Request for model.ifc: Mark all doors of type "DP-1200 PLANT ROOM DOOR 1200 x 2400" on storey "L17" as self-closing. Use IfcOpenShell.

First a look at what the model holds.

```python
import ifcopenshell
import ifcopenshell.util.element

model = ifcopenshell.open("model.ifc")
print(model.schema)
storey = next(s for s in model.by_type("IfcBuildingStorey") if s.Name == "L17")
doors = [e for e in ifcopenshell.util.element.get_decomposition(storey) if e.is_a("IfcDoor")]
seen = {}
for e in doors:
    element_type = ifcopenshell.util.element.get_type(e)
    key = (element_type.Name if element_type != e and element_type else None, ifcopenshell.util.element.get_pset(e, "Pset_DoorCommon", "SelfClosing"))
    seen[key] = seen.get(key, 0) + 1
for (name, value), count in sorted(seen.items(), key=str):
    print(count, "x", name, "|", value)
```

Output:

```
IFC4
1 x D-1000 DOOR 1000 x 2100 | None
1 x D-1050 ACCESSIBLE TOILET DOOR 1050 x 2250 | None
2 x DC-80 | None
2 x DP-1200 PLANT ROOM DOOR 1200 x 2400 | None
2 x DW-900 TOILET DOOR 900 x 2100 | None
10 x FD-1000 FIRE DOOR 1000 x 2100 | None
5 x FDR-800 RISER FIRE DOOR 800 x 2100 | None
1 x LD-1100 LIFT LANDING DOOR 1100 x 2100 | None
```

```python
import ifcopenshell
import ifcopenshell.api.pset
import ifcopenshell.util.element

model = ifcopenshell.open("model.ifc")

storey = next(s for s in model.by_type("IfcBuildingStorey") if s.Name == "L17")
doors = [e for e in ifcopenshell.util.element.get_decomposition(storey) if e.is_a("IfcDoor")]

count = 0
for e in doors:
    element_type = ifcopenshell.util.element.get_type(e)
    if element_type in (None, e) or element_type.Name != "DP-1200 PLANT ROOM DOOR 1200 x 2400":
        continue
    # add_pset returns the element's existing set when there is one.
    pset = ifcopenshell.api.pset.add_pset(model, product=e, name="Pset_DoorCommon")
    ifcopenshell.api.pset.edit_pset(model, pset=pset, properties={"SelfClosing": True})
    count += 1

print(count, "doors updated")

model.write("model_updated.ifc")
```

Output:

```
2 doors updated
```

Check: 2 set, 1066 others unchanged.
